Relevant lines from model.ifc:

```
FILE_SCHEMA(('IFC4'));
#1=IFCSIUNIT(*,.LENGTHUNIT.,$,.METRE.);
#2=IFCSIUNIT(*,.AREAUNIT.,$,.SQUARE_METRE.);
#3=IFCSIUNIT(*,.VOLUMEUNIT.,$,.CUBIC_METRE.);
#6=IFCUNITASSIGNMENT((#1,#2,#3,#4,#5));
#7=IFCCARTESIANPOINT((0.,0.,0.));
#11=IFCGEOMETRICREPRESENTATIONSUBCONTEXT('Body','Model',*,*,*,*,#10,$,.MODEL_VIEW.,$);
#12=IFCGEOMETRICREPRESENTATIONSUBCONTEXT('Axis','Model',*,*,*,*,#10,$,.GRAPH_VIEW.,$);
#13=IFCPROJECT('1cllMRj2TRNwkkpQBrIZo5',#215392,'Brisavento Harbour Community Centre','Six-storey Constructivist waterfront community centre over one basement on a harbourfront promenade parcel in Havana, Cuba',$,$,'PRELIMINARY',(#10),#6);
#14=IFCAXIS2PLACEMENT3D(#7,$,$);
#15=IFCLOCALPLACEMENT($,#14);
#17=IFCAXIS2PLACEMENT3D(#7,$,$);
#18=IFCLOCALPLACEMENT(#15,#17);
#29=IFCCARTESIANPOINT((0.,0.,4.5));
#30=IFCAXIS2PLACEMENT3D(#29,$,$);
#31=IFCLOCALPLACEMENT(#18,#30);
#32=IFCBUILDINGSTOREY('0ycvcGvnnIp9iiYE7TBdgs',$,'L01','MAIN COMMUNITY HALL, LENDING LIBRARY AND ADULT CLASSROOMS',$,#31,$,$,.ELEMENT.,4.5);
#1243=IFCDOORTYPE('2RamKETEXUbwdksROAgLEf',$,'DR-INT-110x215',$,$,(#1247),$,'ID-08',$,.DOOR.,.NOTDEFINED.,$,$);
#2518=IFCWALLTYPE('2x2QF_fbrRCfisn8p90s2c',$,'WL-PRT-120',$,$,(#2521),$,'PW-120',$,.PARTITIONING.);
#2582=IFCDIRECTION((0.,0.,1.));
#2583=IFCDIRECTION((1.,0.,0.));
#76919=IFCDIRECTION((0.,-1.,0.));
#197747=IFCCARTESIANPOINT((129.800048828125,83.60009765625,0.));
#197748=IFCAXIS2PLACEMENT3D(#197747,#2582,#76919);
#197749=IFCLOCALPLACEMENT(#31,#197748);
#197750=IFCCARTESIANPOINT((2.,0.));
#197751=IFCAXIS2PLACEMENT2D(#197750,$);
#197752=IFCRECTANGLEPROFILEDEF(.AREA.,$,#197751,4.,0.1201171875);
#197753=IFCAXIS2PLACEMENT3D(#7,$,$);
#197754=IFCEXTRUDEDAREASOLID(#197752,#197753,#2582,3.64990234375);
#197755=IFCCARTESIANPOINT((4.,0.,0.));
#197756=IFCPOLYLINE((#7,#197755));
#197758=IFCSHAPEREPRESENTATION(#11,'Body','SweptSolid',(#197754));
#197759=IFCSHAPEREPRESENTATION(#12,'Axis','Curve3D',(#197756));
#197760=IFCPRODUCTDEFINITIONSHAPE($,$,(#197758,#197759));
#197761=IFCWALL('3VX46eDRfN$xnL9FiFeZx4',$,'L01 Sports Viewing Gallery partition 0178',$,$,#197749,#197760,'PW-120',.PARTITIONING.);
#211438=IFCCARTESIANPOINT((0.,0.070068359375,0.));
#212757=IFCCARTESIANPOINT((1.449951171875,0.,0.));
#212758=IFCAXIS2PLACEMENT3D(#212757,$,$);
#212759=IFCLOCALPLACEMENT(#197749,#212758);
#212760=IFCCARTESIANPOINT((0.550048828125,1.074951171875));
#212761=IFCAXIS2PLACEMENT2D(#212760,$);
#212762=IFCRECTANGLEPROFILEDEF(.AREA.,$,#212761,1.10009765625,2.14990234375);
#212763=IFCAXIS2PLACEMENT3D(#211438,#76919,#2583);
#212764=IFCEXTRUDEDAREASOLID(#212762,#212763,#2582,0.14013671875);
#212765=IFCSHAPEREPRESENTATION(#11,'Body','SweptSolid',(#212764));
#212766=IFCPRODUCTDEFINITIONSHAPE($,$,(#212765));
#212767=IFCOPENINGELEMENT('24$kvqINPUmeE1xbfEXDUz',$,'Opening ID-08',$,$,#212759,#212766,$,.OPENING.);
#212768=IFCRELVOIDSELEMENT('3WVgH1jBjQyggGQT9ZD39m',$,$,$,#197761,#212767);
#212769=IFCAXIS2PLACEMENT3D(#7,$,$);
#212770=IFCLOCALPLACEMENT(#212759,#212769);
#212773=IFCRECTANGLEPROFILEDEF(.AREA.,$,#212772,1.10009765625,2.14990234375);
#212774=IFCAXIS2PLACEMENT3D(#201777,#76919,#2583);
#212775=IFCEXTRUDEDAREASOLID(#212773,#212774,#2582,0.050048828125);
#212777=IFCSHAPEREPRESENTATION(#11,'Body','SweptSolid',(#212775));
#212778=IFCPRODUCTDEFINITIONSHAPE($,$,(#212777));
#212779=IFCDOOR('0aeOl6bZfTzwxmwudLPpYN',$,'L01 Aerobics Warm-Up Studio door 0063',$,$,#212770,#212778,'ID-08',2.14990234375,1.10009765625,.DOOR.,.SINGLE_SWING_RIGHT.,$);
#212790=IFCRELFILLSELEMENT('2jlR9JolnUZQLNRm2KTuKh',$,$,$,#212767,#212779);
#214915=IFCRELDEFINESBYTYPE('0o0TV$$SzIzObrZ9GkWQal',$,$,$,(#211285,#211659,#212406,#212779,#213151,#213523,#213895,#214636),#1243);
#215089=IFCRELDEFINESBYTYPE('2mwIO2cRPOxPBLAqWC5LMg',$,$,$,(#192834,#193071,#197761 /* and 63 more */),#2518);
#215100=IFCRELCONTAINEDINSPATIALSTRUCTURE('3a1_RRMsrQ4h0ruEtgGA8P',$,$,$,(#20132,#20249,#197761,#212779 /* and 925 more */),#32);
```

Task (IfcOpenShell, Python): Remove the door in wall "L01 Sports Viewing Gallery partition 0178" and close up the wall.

```python
import ifcopenshell
import ifcopenshell.api.feature
import ifcopenshell.api.root
import ifcopenshell.geom
import ifcopenshell.util.shape

model = ifcopenshell.open("model.ifc")
settings = ifcopenshell.geom.settings()


def volume(element):
    """Net volume in cubic metres, openings subtracted."""
    shape = ifcopenshell.geom.create_shape(settings, element)
    return ifcopenshell.util.shape.get_volume(shape.geometry)


door = model.by_id(212779)
opening = door.FillsVoids[0].RelatingOpeningElement
wall = opening.VoidsElements[0].RelatingBuildingElement
before = volume(wall)

ifcopenshell.api.root.remove_product(model, product=door)
ifcopenshell.api.feature.remove_feature(model, feature=opening)

after = volume(wall)

print(f"wall volume {before:.3f} -> {after:.3f} m3")

model.write("model_updated.ifc")
```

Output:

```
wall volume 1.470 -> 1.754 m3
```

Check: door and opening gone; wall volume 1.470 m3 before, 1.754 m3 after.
